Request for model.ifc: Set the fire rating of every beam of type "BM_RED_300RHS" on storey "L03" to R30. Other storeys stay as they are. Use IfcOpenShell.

First a look at what the model holds.

```python
import ifcopenshell
import ifcopenshell.util.element

model = ifcopenshell.open("model.ifc")
print(model.schema)
storey = next(s for s in model.by_type("IfcBuildingStorey") if s.Name == "L03")
beams = [e for e in ifcopenshell.util.element.get_decomposition(storey) if e.is_a("IfcBeam")]
seen = {}
for e in beams:
    element_type = ifcopenshell.util.element.get_type(e)
    key = (element_type.Name if element_type != e and element_type else None, ifcopenshell.util.element.get_pset(e, "Pset_BeamCommon", "FireRating"))
    seen[key] = seen.get(key, 0) + 1
for (name, value), count in sorted(seen.items(), key=str):
    print(count, "x", name, "|", value)
```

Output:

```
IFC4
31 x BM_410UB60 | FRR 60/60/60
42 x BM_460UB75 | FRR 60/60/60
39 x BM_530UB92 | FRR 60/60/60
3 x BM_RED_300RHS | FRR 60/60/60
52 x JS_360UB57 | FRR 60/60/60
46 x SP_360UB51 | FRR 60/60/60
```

```python
import ifcopenshell
import ifcopenshell.api.pset
import ifcopenshell.util.element

model = ifcopenshell.open("model.ifc")

storey = next(s for s in model.by_type("IfcBuildingStorey") if s.Name == "L03")
beams = [e for e in ifcopenshell.util.element.get_decomposition(storey) if e.is_a("IfcBeam")]

count = 0
for e in beams:
    element_type = ifcopenshell.util.element.get_type(e)
    if element_type in (None, e) or element_type.Name != "BM_RED_300RHS":
        continue
    # add_pset returns the element's existing set when there is one.
    pset = ifcopenshell.api.pset.add_pset(model, product=e, name="Pset_BeamCommon")
    ifcopenshell.api.pset.edit_pset(model, pset=pset, properties={"FireRating": "R30"})
    count += 1

print(count, "beams updated")

model.write("model_rev.ifc")
```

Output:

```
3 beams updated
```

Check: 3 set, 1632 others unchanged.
